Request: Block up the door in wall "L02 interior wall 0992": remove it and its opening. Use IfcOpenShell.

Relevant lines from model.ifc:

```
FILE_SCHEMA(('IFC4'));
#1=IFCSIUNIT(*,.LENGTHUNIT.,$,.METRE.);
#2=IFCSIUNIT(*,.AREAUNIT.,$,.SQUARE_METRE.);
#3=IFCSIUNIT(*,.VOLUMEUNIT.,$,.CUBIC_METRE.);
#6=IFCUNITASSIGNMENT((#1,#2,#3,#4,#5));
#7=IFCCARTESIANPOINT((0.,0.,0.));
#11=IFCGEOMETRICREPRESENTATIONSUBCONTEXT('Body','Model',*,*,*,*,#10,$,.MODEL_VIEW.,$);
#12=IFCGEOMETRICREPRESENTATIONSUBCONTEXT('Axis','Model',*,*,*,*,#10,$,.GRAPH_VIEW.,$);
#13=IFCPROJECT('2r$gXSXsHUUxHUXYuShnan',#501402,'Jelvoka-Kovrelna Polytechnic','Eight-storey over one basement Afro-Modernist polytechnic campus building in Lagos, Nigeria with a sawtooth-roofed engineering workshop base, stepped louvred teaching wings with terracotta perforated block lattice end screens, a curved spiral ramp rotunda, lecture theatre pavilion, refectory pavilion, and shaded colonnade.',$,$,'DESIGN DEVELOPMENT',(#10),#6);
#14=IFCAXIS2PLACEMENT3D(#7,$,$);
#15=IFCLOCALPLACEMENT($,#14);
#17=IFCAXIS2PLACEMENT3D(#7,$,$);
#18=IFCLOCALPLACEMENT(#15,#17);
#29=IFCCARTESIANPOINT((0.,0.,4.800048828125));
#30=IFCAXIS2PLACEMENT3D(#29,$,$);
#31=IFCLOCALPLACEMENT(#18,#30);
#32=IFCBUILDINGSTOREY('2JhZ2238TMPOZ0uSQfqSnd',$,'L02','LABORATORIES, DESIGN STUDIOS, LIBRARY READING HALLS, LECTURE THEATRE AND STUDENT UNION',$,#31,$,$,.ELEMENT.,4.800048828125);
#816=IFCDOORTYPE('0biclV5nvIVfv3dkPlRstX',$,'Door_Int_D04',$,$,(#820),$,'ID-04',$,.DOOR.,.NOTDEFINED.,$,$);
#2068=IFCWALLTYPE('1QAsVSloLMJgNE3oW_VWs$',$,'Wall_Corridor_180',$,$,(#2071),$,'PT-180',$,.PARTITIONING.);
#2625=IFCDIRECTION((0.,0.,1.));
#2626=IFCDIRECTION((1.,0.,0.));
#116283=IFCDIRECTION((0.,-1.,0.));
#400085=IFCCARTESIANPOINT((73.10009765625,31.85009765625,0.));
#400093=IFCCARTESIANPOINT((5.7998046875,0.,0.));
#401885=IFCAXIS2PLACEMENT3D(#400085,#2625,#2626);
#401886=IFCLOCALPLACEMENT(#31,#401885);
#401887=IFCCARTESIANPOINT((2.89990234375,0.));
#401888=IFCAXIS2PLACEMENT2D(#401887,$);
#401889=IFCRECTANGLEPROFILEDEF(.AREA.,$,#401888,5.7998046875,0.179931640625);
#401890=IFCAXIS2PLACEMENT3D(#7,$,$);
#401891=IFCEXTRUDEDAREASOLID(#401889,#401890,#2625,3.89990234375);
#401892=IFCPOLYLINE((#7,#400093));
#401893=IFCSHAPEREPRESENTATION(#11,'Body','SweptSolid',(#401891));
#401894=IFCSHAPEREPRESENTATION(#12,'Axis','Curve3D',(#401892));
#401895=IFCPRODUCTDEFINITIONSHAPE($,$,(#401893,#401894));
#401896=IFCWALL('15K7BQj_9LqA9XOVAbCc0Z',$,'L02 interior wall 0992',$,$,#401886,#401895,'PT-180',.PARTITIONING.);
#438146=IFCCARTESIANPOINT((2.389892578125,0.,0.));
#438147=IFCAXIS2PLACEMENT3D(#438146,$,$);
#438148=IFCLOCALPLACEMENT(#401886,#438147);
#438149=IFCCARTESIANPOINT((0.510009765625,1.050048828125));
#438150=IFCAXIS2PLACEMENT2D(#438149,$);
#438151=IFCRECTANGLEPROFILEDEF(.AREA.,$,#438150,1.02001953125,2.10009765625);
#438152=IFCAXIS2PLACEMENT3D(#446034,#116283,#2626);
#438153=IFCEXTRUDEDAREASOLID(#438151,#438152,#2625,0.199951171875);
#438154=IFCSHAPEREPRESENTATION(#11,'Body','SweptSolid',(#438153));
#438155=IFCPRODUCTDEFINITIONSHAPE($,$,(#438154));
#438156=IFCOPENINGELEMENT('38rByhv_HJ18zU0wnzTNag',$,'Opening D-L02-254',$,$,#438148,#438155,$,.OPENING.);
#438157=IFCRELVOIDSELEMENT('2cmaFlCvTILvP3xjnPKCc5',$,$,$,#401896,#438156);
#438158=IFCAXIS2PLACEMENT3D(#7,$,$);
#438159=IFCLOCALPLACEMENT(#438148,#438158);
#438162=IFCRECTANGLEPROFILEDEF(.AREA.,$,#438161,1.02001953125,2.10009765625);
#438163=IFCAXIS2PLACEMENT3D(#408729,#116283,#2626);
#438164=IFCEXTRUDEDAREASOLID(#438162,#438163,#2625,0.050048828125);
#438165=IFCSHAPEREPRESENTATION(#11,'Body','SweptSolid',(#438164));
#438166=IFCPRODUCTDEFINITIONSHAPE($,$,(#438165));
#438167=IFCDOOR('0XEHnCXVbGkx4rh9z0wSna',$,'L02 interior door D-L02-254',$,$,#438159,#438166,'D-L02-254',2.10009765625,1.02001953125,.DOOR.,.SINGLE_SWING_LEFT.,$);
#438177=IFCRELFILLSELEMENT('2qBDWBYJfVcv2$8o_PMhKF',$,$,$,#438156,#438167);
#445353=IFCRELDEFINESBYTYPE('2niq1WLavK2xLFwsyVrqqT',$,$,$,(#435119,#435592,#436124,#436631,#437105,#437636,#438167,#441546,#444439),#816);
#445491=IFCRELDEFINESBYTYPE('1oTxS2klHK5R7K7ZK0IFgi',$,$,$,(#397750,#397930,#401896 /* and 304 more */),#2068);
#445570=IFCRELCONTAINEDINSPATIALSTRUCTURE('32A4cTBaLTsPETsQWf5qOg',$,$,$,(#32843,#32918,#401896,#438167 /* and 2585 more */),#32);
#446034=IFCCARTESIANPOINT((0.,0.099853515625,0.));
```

```python
import ifcopenshell
import ifcopenshell.api.feature
import ifcopenshell.api.root
import ifcopenshell.geom
import ifcopenshell.util.shape

model = ifcopenshell.open("model.ifc")
settings = ifcopenshell.geom.settings()


def volume(element):
    """Net volume in cubic metres, openings subtracted."""
    shape = ifcopenshell.geom.create_shape(settings, element)
    return ifcopenshell.util.shape.get_volume(shape.geometry)


door = model.by_id(438167)
opening = door.FillsVoids[0].RelatingOpeningElement
wall = opening.VoidsElements[0].RelatingBuildingElement
before = volume(wall)

ifcopenshell.api.root.remove_product(model, product=door)
ifcopenshell.api.feature.remove_feature(model, feature=opening)

after = volume(wall)

print(f"wall volume {before:.3f} -> {after:.3f} m3")

model.write("model_edited.ifc")
```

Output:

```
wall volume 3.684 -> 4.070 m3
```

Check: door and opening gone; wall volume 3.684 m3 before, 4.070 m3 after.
